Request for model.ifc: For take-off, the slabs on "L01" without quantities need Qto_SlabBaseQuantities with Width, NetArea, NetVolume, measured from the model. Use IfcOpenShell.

First a look at what the model holds.

```python
import ifcopenshell
import ifcopenshell.util.element
import ifcopenshell.util.unit

model = ifcopenshell.open("model.ifc")
print(model.schema)
for unit_type in ("LENGTHUNIT", "AREAUNIT", "VOLUMEUNIT"):
    print(unit_type, ifcopenshell.util.unit.calculate_unit_scale(model, unit_type))
storey = next(s for s in model.by_type("IfcBuildingStorey") if s.Name == "L01")
slabs = [e for e in ifcopenshell.util.element.get_decomposition(storey) if e.is_a("IfcSlab")]
for e in sorted(slabs, key=lambda e: e.id()):
    print(e.id(), e.is_a(), e.Name, list(ifcopenshell.util.element.get_psets(e, qtos_only=True)), sep=" | ")
```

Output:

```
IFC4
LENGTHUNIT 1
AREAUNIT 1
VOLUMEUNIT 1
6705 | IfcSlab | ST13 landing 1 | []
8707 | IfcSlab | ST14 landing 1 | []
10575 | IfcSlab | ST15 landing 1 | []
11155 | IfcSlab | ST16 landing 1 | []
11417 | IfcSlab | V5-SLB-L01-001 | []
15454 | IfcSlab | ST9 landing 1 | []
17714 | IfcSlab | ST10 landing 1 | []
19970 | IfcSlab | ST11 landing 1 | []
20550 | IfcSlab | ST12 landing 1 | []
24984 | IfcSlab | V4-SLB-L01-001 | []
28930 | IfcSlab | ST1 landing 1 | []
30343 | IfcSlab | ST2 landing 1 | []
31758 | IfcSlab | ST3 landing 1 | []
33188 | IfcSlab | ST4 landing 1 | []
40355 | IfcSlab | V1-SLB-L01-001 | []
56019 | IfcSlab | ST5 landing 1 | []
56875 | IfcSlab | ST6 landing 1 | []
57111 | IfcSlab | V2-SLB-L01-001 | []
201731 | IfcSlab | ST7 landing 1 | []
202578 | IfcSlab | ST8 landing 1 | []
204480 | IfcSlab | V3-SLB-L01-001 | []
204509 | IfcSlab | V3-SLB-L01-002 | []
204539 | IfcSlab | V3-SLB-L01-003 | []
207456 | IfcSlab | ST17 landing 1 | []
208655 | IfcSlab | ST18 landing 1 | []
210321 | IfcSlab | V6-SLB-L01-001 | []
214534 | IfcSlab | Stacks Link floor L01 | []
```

```python
import ifcopenshell
import ifcopenshell.api.pset
import ifcopenshell.geom
import ifcopenshell.util.element
import ifcopenshell.util.shape
import ifcopenshell.util.unit

model = ifcopenshell.open("model.ifc")
unit_scale = ifcopenshell.util.unit.calculate_unit_scale(model)
area_scale = ifcopenshell.util.unit.calculate_unit_scale(model, "AREAUNIT")
volume_scale = ifcopenshell.util.unit.calculate_unit_scale(model, "VOLUMEUNIT")
settings = ifcopenshell.geom.settings()

storey = next(s for s in model.by_type("IfcBuildingStorey") if s.Name == "L01")
slabs = [e for e in ifcopenshell.util.element.get_decomposition(storey) if e.is_a("IfcSlab")]

for e in sorted(slabs, key=lambda e: e.id()):
    if ifcopenshell.util.element.get_psets(e, qtos_only=True, should_inherit=False):
        continue
    # Geometry comes back in metres, in the element's own axes.
    shape = ifcopenshell.geom.create_shape(settings, e)
    values = {
        "Width": ifcopenshell.util.shape.get_z(shape.geometry) / unit_scale,
        "NetArea": ifcopenshell.util.shape.get_footprint_area(shape.geometry) / area_scale,
        "NetVolume": ifcopenshell.util.shape.get_volume(shape.geometry) / volume_scale,
    }
    qto = ifcopenshell.api.pset.add_qto(model, product=e, name="Qto_SlabBaseQuantities")
    ifcopenshell.api.pset.edit_qto(model, qto=qto, properties=values)
    print(e.id(), {k: round(v, 3) for k, v in values.items()})

model.write("model-out.ifc")
```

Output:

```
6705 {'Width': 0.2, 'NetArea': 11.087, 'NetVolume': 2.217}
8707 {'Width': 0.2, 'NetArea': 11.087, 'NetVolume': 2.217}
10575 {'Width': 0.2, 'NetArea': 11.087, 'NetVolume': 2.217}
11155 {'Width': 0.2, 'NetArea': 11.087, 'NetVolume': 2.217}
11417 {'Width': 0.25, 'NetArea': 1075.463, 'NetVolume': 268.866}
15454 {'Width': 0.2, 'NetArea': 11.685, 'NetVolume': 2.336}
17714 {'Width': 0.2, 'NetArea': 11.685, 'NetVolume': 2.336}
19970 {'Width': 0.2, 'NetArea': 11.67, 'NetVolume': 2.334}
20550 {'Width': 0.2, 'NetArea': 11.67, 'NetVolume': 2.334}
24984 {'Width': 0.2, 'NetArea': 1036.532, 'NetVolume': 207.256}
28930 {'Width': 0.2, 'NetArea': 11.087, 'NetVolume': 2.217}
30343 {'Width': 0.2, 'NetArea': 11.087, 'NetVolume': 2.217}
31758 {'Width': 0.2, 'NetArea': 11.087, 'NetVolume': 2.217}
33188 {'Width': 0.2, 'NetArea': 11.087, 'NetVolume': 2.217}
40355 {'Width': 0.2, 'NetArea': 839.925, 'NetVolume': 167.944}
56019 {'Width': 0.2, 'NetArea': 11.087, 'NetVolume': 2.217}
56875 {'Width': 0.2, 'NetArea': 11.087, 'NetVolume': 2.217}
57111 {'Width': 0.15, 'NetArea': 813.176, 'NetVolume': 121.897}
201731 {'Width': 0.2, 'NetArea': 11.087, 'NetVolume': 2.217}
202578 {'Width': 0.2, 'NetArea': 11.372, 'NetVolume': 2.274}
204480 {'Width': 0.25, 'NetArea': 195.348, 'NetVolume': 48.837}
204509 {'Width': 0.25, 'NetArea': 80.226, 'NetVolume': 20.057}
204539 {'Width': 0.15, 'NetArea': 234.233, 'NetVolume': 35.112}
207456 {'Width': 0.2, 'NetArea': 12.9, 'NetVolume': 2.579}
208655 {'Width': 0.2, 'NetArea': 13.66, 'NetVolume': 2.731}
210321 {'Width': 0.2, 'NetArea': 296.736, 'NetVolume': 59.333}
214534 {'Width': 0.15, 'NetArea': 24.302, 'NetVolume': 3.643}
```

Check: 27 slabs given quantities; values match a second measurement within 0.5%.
